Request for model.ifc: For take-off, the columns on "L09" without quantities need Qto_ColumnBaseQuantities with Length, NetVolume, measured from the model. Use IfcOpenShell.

First a look at what the model holds.

```python
import ifcopenshell
import ifcopenshell.util.element
import ifcopenshell.util.unit

model = ifcopenshell.open("model.ifc")
print(model.schema)
for unit_type in ("LENGTHUNIT", "AREAUNIT", "VOLUMEUNIT"):
    print(unit_type, ifcopenshell.util.unit.calculate_unit_scale(model, unit_type))
storey = next(s for s in model.by_type("IfcBuildingStorey") if s.Name == "L09")
columns = [e for e in ifcopenshell.util.element.get_decomposition(storey) if e.is_a("IfcColumn")]
for e in sorted(columns, key=lambda e: e.id()):
    print(e.id(), e.is_a(), e.Name, list(ifcopenshell.util.element.get_psets(e, qtos_only=True)), sep=" | ")
```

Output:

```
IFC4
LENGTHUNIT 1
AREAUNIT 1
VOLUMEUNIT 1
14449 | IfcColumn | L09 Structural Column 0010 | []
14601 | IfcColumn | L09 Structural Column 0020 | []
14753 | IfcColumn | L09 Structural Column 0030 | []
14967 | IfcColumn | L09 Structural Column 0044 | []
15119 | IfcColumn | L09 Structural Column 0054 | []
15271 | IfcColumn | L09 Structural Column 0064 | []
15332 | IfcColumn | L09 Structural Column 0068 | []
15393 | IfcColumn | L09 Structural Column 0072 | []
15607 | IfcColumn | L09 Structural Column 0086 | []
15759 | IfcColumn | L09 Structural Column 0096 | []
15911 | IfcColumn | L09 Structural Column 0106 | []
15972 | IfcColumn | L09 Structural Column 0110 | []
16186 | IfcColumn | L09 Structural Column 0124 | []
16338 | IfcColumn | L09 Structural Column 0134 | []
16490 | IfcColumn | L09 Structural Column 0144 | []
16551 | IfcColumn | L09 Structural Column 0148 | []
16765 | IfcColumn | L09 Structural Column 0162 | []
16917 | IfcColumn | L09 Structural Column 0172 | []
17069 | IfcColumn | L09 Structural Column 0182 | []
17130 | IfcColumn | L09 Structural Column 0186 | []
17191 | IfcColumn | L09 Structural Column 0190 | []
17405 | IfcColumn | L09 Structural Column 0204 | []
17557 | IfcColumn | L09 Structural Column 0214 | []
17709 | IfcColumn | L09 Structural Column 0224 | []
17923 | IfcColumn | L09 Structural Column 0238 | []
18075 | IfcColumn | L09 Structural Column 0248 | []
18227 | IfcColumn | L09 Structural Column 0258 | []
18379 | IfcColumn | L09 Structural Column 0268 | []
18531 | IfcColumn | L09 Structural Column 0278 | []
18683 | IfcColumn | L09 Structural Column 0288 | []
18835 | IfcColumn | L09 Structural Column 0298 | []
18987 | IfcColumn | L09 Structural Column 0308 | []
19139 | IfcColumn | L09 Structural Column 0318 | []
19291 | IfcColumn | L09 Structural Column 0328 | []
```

```python
import ifcopenshell
import ifcopenshell.api.pset
import ifcopenshell.geom
import ifcopenshell.util.element
import ifcopenshell.util.shape
import ifcopenshell.util.unit

model = ifcopenshell.open("model.ifc")
unit_scale = ifcopenshell.util.unit.calculate_unit_scale(model)
volume_scale = ifcopenshell.util.unit.calculate_unit_scale(model, "VOLUMEUNIT")
settings = ifcopenshell.geom.settings()

storey = next(s for s in model.by_type("IfcBuildingStorey") if s.Name == "L09")
columns = [e for e in ifcopenshell.util.element.get_decomposition(storey) if e.is_a("IfcColumn")]

for e in sorted(columns, key=lambda e: e.id()):
    if ifcopenshell.util.element.get_psets(e, qtos_only=True, should_inherit=False):
        continue
    # Geometry comes back in metres, in the element's own axes.
    shape = ifcopenshell.geom.create_shape(settings, e)
    values = {
        "Length": ifcopenshell.util.shape.get_z(shape.geometry) / unit_scale,
        "NetVolume": ifcopenshell.util.shape.get_volume(shape.geometry) / volume_scale,
    }
    qto = ifcopenshell.api.pset.add_qto(model, product=e, name="Qto_ColumnBaseQuantities")
    ifcopenshell.api.pset.edit_qto(model, qto=qto, properties=values)
    print(e.id(), {k: round(v, 3) for k, v in values.items()})

model.write("model_rev.ifc")
```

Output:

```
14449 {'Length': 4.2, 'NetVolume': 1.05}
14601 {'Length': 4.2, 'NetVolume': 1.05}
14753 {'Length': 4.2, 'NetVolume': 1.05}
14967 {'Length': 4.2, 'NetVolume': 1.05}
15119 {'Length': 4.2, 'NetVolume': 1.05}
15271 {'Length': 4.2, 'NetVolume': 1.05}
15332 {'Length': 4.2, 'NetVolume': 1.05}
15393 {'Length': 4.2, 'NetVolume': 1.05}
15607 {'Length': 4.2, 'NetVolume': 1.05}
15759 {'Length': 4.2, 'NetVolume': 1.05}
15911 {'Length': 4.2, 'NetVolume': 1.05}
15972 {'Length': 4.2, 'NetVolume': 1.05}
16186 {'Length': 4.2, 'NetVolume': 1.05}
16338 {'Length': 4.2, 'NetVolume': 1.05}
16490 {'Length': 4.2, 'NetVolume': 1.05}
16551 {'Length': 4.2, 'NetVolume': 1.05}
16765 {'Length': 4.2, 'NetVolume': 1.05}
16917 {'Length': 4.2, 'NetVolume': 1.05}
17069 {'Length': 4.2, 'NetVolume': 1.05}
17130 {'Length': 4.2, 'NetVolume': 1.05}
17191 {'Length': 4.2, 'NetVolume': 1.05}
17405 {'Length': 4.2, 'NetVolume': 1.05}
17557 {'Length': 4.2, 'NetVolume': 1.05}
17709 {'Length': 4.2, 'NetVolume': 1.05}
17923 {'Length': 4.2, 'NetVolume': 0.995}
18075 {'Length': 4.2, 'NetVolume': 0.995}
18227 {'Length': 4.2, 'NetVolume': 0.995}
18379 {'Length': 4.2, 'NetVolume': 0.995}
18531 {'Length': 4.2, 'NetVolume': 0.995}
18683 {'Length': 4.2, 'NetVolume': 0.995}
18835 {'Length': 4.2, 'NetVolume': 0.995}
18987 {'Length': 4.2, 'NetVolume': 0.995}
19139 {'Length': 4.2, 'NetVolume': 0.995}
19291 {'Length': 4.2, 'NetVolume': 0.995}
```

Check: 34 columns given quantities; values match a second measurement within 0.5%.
